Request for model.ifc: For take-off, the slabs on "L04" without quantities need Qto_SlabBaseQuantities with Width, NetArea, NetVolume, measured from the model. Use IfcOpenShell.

First a look at what the model holds.

```python
import ifcopenshell
import ifcopenshell.util.element
import ifcopenshell.util.unit

model = ifcopenshell.open("model.ifc")
print(model.schema)
for unit_type in ("LENGTHUNIT", "AREAUNIT", "VOLUMEUNIT"):
    print(unit_type, ifcopenshell.util.unit.calculate_unit_scale(model, unit_type))
storey = next(s for s in model.by_type("IfcBuildingStorey") if s.Name == "L04")
slabs = [e for e in ifcopenshell.util.element.get_decomposition(storey) if e.is_a("IfcSlab")]
for e in sorted(slabs, key=lambda e: e.id()):
    print(e.id(), e.is_a(), e.Name, list(ifcopenshell.util.element.get_psets(e, qtos_only=True)), sep=" | ")
```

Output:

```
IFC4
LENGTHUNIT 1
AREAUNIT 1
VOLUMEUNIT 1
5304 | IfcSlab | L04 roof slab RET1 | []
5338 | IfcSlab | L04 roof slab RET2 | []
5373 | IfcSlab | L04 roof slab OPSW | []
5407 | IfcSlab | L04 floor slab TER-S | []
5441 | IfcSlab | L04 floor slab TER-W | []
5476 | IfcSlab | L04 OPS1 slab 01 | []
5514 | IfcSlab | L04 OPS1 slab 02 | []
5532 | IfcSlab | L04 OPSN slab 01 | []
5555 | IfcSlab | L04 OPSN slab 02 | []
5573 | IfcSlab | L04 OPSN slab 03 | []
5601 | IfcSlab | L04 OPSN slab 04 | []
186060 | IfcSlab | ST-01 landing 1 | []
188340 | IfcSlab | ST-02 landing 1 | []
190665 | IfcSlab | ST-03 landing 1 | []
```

```python
import ifcopenshell
import ifcopenshell.api.pset
import ifcopenshell.geom
import ifcopenshell.util.element
import ifcopenshell.util.shape
import ifcopenshell.util.unit

model = ifcopenshell.open("model.ifc")
unit_scale = ifcopenshell.util.unit.calculate_unit_scale(model)
area_scale = ifcopenshell.util.unit.calculate_unit_scale(model, "AREAUNIT")
volume_scale = ifcopenshell.util.unit.calculate_unit_scale(model, "VOLUMEUNIT")
settings = ifcopenshell.geom.settings()

storey = next(s for s in model.by_type("IfcBuildingStorey") if s.Name == "L04")
slabs = [e for e in ifcopenshell.util.element.get_decomposition(storey) if e.is_a("IfcSlab")]

for e in sorted(slabs, key=lambda e: e.id()):
    if ifcopenshell.util.element.get_psets(e, qtos_only=True, should_inherit=False):
        continue
    # Geometry comes back in metres, in the element's own axes.
    shape = ifcopenshell.geom.create_shape(settings, e)
    values = {
        "Width": ifcopenshell.util.shape.get_z(shape.geometry) / unit_scale,
        "NetArea": ifcopenshell.util.shape.get_footprint_area(shape.geometry) / area_scale,
        "NetVolume": ifcopenshell.util.shape.get_volume(shape.geometry) / volume_scale,
    }
    qto = ifcopenshell.api.pset.add_qto(model, product=e, name="Qto_SlabBaseQuantities")
    ifcopenshell.api.pset.edit_qto(model, qto=qto, properties=values)
    print(e.id(), {k: round(v, 3) for k, v in values.items()})

model.write("model_edited.ifc")
```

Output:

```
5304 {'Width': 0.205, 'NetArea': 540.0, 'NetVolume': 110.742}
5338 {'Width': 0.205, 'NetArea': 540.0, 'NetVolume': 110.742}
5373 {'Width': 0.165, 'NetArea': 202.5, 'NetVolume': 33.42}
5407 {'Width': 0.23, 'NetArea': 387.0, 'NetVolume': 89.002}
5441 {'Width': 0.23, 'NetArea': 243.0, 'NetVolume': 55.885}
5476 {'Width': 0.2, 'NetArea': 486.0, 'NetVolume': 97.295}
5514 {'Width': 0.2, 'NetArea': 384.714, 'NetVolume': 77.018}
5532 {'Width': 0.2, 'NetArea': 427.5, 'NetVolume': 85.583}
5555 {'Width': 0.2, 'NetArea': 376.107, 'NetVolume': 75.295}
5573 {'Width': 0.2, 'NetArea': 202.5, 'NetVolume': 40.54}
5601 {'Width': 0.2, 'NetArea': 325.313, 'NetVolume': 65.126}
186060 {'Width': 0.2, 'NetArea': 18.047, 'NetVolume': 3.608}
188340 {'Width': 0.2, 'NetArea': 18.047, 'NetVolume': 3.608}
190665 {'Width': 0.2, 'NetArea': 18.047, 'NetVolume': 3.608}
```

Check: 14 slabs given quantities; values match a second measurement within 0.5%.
